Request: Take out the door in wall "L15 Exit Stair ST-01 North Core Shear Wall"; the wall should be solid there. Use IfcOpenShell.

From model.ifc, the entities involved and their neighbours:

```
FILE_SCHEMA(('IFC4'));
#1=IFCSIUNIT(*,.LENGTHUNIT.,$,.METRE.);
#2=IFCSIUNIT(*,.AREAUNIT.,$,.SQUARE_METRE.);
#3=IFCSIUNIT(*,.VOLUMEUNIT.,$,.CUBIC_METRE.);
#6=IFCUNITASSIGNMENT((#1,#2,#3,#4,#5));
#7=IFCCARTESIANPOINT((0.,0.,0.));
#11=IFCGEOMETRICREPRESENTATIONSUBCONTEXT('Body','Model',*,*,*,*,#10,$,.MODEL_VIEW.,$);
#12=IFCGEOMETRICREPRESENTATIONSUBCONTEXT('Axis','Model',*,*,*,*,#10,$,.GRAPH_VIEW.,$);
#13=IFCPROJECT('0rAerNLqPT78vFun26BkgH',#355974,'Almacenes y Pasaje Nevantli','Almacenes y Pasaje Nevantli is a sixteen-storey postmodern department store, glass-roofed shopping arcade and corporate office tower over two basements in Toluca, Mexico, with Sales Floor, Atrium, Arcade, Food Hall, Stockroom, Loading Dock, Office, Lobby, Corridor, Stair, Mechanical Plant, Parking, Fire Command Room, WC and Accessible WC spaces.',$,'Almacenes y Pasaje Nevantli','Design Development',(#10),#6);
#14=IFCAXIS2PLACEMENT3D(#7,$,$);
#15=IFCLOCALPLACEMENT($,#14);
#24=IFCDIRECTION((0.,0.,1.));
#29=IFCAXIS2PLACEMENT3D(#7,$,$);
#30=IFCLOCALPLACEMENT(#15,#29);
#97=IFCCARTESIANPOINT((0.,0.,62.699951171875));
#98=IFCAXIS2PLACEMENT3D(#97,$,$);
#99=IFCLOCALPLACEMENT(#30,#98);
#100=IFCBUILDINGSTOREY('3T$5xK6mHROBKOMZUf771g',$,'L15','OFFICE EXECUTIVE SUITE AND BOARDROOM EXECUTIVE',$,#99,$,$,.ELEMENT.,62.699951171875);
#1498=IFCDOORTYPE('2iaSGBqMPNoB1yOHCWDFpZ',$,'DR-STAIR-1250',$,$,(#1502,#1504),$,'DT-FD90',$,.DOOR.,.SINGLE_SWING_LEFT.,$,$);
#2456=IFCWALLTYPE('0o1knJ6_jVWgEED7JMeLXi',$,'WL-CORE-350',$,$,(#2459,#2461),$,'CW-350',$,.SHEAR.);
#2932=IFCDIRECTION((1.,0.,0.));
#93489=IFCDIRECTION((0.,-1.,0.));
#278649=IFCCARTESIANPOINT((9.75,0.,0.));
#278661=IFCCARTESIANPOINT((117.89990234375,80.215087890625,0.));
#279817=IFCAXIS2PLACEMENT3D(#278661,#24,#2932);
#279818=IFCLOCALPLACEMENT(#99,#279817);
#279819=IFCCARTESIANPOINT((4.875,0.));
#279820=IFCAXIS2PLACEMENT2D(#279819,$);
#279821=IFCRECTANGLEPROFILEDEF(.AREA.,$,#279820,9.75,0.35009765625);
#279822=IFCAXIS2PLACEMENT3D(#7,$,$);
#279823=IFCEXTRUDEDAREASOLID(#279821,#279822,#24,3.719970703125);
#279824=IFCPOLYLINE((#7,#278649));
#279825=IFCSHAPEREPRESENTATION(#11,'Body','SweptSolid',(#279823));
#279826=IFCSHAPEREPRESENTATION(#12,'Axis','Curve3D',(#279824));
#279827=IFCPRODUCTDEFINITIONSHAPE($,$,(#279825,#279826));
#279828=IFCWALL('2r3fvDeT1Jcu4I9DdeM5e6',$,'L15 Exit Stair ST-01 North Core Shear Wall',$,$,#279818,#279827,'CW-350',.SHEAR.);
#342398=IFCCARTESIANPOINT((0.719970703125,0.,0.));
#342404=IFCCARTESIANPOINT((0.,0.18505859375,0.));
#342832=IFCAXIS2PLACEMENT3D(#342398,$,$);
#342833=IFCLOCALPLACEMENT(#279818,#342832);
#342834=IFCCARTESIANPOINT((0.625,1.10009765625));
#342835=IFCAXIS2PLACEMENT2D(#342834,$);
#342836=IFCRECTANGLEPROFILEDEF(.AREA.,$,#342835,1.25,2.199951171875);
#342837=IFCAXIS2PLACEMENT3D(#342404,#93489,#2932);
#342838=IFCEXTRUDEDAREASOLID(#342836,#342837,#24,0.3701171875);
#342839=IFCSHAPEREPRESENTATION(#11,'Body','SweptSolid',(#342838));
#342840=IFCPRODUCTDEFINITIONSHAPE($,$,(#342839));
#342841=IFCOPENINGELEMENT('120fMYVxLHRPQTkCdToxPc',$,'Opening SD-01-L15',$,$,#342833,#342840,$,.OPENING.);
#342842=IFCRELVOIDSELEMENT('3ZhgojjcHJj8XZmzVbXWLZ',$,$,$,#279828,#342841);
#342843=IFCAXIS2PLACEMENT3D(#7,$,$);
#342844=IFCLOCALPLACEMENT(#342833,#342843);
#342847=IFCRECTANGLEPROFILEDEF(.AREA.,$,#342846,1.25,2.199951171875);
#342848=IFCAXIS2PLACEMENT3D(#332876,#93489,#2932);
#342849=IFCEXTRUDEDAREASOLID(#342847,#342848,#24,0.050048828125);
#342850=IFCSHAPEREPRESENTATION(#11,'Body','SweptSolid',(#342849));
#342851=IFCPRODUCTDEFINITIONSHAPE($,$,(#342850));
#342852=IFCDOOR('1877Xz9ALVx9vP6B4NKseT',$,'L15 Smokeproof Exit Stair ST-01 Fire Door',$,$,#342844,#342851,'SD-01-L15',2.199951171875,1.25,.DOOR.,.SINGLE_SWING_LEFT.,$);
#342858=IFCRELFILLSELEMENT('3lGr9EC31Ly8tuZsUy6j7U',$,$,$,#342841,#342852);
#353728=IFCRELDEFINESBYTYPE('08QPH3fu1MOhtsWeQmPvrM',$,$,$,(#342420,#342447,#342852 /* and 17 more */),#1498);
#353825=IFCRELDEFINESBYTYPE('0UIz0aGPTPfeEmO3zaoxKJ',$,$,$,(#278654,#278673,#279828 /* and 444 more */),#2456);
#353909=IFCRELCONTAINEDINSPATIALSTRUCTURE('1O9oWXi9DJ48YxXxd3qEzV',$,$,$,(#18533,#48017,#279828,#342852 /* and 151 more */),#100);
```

```python
import ifcopenshell
import ifcopenshell.api.feature
import ifcopenshell.api.root
import ifcopenshell.geom
import ifcopenshell.util.shape

model = ifcopenshell.open("model.ifc")
settings = ifcopenshell.geom.settings()


def volume(element):
    """Net volume in cubic metres, openings subtracted."""
    shape = ifcopenshell.geom.create_shape(settings, element)
    return ifcopenshell.util.shape.get_volume(shape.geometry)


door = model.by_guid("1877Xz9ALVx9vP6B4NKseT")
opening = door.FillsVoids[0].RelatingOpeningElement
wall = opening.VoidsElements[0].RelatingBuildingElement
before = volume(wall)

ifcopenshell.api.root.remove_product(model, product=door)
ifcopenshell.api.feature.remove_feature(model, feature=opening)

after = volume(wall)

print(f"wall volume {before:.3f} -> {after:.3f} m3")

model.write("model_edited.ifc")
```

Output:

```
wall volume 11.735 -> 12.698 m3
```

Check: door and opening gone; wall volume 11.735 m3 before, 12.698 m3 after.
